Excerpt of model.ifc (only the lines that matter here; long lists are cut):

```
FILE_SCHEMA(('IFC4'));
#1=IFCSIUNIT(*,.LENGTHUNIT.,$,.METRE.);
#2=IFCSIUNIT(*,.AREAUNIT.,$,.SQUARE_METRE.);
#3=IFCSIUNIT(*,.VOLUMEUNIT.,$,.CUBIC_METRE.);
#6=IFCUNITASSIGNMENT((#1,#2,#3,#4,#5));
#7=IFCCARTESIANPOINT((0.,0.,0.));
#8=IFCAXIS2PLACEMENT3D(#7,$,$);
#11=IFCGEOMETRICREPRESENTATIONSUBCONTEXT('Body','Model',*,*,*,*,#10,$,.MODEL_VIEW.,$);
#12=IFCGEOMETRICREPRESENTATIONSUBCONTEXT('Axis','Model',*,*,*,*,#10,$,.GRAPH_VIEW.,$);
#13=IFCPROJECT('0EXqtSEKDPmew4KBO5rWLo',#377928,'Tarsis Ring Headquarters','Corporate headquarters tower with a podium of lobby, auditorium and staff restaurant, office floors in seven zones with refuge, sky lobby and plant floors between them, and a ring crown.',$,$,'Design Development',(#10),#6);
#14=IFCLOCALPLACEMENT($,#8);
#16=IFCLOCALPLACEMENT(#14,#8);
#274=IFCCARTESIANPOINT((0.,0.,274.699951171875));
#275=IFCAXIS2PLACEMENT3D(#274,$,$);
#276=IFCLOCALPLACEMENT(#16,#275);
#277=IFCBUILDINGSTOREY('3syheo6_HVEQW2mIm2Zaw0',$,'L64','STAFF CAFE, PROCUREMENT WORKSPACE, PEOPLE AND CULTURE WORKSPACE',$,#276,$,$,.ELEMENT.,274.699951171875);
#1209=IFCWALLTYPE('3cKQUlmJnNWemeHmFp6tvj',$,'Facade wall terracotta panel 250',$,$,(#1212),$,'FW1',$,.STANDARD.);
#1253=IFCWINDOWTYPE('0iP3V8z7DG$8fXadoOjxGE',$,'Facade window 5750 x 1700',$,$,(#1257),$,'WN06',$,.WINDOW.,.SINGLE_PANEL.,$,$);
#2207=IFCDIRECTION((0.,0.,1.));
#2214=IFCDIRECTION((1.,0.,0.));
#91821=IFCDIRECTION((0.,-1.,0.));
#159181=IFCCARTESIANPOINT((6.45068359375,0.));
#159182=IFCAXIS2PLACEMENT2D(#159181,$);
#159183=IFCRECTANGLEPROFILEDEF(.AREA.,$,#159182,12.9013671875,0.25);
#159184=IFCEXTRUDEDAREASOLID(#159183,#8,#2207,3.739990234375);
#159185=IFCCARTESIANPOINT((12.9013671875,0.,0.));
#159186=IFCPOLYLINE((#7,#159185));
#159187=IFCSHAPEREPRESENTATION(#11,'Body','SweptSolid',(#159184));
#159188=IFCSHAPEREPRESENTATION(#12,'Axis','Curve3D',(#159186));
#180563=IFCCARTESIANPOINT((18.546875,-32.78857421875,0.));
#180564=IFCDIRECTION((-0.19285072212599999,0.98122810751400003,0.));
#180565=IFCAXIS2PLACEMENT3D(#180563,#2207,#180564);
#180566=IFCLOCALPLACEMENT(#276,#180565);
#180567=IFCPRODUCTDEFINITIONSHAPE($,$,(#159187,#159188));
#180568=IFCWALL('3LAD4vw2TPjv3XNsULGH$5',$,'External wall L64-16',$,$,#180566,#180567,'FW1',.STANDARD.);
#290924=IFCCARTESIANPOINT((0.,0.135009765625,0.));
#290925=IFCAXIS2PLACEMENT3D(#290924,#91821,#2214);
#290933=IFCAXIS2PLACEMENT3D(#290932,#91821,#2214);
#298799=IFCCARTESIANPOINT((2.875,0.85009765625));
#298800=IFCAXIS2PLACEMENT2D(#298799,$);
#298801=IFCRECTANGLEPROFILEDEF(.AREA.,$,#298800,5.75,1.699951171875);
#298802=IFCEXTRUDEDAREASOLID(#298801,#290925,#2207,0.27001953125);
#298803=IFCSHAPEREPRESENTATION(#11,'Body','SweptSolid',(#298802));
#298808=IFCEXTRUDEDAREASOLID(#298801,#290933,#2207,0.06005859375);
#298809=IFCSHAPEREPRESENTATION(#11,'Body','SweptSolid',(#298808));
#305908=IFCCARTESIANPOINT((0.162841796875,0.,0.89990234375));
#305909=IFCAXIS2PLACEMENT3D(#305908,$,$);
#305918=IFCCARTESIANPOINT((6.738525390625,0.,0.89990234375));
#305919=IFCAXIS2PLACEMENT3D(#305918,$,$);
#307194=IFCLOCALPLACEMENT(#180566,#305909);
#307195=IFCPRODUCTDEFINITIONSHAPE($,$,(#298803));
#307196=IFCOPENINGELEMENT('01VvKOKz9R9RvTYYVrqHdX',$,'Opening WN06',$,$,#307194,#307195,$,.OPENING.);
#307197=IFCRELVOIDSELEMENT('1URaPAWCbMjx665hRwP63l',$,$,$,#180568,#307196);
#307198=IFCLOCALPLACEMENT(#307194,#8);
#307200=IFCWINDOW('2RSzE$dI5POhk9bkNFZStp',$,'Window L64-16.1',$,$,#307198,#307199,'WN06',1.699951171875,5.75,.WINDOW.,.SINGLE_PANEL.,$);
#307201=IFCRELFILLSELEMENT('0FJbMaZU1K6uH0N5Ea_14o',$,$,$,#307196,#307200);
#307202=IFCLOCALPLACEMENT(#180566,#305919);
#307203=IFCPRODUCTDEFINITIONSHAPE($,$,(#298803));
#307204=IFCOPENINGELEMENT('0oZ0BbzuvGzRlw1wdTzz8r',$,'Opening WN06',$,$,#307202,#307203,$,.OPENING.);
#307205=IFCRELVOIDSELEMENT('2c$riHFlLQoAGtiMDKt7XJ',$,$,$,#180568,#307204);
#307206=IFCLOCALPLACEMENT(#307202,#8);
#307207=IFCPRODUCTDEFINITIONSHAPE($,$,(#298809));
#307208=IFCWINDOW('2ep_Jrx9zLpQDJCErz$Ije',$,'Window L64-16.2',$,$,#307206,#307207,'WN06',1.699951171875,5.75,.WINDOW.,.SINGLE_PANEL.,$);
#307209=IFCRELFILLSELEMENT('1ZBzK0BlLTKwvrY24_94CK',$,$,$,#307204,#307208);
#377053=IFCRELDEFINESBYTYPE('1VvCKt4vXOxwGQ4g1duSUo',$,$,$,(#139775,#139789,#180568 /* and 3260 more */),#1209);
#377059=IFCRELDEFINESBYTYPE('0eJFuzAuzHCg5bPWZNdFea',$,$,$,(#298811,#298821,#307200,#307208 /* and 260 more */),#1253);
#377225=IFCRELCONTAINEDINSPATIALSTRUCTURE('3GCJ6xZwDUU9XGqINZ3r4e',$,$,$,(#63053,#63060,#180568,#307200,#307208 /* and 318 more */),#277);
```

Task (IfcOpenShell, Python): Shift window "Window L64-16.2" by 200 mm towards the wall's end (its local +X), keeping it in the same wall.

```python
import ifcopenshell
import ifcopenshell.api.geometry
import ifcopenshell.util.placement

model = ifcopenshell.open("model.ifc")

window = model.by_guid("2ep_Jrx9zLpQDJCErz$Ije")
opening = window.FillsVoids[0].RelatingOpeningElement
wall = opening.VoidsElements[0].RelatingBuildingElement

wall_matrix = ifcopenshell.util.placement.get_local_placement(wall.ObjectPlacement)
shift = wall_matrix[:3, 0] * 0.2
before = ifcopenshell.util.placement.get_local_placement(window.ObjectPlacement)[:3, 3].copy()

# The window is placed relative to its opening, so it follows when the opening moves.
matrix = ifcopenshell.util.placement.get_local_placement(opening.ObjectPlacement)
matrix[:3, 3] += shift
ifcopenshell.api.geometry.edit_object_placement(
    model, product=opening, matrix=matrix, is_si=False, should_transform_children=True
)

after = ifcopenshell.util.placement.get_local_placement(window.ObjectPlacement)[:3, 3]
print("window moved by", (after - before).round(3) + 0.0)

model.write("model_rev.ifc")
```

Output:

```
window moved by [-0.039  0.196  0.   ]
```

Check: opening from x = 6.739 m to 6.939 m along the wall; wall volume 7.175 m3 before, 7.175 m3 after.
